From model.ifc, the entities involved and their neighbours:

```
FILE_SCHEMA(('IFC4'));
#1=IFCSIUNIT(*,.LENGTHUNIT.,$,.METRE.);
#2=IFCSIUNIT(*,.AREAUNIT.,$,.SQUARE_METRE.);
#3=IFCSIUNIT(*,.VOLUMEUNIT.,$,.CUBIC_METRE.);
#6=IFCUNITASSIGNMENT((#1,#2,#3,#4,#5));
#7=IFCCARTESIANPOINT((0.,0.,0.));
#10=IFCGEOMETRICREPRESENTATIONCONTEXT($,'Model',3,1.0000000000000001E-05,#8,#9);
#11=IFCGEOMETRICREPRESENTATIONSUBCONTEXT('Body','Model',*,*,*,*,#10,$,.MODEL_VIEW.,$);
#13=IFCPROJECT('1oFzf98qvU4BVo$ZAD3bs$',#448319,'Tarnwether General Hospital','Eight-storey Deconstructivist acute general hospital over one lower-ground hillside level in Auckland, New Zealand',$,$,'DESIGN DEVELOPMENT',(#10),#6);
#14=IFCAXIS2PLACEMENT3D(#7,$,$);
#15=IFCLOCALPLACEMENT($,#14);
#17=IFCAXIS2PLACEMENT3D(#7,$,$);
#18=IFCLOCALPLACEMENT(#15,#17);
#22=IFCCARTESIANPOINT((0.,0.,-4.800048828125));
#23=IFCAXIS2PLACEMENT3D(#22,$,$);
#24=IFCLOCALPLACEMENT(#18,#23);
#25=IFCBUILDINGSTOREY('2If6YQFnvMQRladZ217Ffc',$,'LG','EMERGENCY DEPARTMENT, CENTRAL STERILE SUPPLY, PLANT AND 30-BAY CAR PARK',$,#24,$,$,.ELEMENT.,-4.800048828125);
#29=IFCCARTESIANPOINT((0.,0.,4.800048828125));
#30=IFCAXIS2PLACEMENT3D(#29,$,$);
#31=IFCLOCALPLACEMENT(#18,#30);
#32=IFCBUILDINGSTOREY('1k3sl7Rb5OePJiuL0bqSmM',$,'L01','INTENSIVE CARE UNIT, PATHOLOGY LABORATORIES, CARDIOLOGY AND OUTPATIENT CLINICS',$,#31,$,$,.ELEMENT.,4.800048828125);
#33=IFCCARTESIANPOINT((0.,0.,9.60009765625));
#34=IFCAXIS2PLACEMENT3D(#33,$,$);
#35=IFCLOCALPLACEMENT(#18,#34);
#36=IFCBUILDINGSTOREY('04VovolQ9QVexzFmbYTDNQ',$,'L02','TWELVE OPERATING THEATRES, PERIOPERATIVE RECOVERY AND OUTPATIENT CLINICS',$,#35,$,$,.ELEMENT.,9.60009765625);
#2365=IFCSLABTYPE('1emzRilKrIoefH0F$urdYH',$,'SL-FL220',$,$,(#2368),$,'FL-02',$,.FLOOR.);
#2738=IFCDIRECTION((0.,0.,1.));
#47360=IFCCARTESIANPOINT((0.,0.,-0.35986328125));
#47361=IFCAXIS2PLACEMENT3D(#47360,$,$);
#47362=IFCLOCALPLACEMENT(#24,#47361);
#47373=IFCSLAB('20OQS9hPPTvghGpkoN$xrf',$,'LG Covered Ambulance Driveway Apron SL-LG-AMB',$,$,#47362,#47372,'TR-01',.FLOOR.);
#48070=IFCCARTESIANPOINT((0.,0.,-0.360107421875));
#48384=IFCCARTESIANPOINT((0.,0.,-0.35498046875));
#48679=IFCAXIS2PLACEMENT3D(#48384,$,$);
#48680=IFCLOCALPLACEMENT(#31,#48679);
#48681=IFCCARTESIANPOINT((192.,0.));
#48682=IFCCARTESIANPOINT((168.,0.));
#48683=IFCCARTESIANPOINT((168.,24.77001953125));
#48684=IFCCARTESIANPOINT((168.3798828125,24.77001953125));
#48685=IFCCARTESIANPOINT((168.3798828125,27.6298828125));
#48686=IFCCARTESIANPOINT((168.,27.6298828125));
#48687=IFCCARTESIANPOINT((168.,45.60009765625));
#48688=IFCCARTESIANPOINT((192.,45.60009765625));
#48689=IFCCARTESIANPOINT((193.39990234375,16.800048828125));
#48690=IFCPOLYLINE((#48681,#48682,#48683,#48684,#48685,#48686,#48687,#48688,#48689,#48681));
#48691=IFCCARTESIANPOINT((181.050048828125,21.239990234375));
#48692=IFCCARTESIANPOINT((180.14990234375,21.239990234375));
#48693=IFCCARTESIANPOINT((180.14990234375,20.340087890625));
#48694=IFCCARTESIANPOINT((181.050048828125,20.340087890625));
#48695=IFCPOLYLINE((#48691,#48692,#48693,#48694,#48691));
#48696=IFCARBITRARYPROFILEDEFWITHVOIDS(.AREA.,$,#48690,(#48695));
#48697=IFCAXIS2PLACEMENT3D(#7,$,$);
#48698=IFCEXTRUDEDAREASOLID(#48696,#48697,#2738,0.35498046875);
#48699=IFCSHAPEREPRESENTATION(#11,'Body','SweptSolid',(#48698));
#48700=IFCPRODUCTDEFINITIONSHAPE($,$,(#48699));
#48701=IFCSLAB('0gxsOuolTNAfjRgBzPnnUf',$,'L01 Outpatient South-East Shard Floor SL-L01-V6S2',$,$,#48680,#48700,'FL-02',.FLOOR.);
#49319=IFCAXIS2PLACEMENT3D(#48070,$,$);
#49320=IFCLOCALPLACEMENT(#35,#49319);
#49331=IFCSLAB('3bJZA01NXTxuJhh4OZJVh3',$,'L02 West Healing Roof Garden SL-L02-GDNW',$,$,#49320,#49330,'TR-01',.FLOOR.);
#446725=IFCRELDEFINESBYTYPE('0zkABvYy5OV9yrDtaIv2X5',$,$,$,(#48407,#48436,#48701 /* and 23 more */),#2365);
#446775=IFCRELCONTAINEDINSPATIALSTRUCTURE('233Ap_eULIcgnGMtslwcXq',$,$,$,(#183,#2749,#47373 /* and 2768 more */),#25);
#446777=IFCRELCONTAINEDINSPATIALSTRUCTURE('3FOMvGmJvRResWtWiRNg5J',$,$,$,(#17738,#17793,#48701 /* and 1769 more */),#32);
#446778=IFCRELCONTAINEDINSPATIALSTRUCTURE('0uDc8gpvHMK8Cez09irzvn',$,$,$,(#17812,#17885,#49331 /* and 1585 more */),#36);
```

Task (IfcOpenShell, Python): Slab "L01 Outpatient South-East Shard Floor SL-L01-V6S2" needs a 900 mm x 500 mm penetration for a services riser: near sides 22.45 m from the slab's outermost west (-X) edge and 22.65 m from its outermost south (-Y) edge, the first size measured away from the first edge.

```python
import numpy as np
import ifcopenshell
import ifcopenshell.api.feature
import ifcopenshell.api.geometry
import ifcopenshell.api.root
import ifcopenshell.geom
import ifcopenshell.util.placement
import ifcopenshell.util.representation
import ifcopenshell.util.shape
import ifcopenshell.util.unit

model = ifcopenshell.open("model.ifc")
unit_scale = ifcopenshell.util.unit.calculate_unit_scale(model)
settings = ifcopenshell.geom.settings()


def volume(element):
    """Net volume in cubic metres, openings subtracted."""
    shape = ifcopenshell.geom.create_shape(settings, element)
    return ifcopenshell.util.shape.get_volume(shape.geometry)


slab = model.by_id(48701)
before = volume(slab)

# Extent in the slab's own axes, in metres. The edges named are its -X and -Y sides.
slab_shape = ifcopenshell.geom.create_shape(settings, slab)
vertices = ifcopenshell.util.shape.get_vertices(slab_shape.geometry)
x_min, y_min, bottom = vertices.min(axis=0)
top = vertices[:, 2].max()

opening = ifcopenshell.api.root.create_entity(model, ifc_class="IfcOpeningElement", name="Services riser opening", predefined_type="OPENING")
context = ifcopenshell.util.representation.get_context(model, "Model", "Body", "MODEL_VIEW")
width, depth = 0.9, 0.5
outline = [(0.0, 0.0), (width, 0.0), (width, depth), (0.0, depth), (0.0, 0.0)]
# Overshoot both faces by 50 mm so the cut is clean.
shape = ifcopenshell.api.geometry.add_slab_representation(
    model, context=context, depth=top - bottom + 0.1, polyline=outline
)
ifcopenshell.api.geometry.assign_representation(model, product=opening, representation=shape)

matrix = ifcopenshell.util.placement.get_local_placement(slab.ObjectPlacement)
matrix[:, 3] = matrix @ np.append(np.array([x_min + 22.45, y_min + 22.65, bottom - 0.05]) / unit_scale, 1.0)
ifcopenshell.api.geometry.edit_object_placement(model, product=opening, matrix=matrix, is_si=False)
ifcopenshell.api.feature.add_feature(model, feature=opening, element=slab)

after = volume(slab)

print(f"slab volume {before:.3f} -> {after:.3f} m3")

model.write("model_updated.ifc")
```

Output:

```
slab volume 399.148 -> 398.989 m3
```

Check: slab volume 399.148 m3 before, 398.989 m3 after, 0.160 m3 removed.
